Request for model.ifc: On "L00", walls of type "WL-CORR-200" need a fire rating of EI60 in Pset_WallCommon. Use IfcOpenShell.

First a look at what the model holds.

```python
import ifcopenshell
import ifcopenshell.util.element

model = ifcopenshell.open("model.ifc")
print(model.schema)
storey = next(s for s in model.by_type("IfcBuildingStorey") if s.Name == "L00")
walls = [e for e in ifcopenshell.util.element.get_decomposition(storey) if e.is_a("IfcWall")]
seen = {}
for e in walls:
    element_type = ifcopenshell.util.element.get_type(e)
    key = (element_type.Name if element_type != e and element_type else None, ifcopenshell.util.element.get_pset(e, "Pset_WallCommon", "FireRating"))
    seen[key] = seen.get(key, 0) + 1
for (name, value), count in sorted(seen.items(), key=str):
    print(count, "x", name, "|", value)
```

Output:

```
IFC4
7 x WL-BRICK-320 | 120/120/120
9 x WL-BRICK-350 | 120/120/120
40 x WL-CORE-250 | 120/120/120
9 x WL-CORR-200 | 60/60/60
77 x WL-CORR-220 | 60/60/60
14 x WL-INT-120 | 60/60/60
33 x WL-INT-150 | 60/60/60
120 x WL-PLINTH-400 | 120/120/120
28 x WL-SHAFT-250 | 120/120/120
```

```python
import ifcopenshell
import ifcopenshell.api.pset
import ifcopenshell.util.element

model = ifcopenshell.open("model.ifc")

storey = next(s for s in model.by_type("IfcBuildingStorey") if s.Name == "L00")
walls = [e for e in ifcopenshell.util.element.get_decomposition(storey) if e.is_a("IfcWall")]

count = 0
for e in walls:
    element_type = ifcopenshell.util.element.get_type(e)
    if element_type in (None, e) or element_type.Name != "WL-CORR-200":
        continue
    # add_pset returns the element's existing set when there is one.
    pset = ifcopenshell.api.pset.add_pset(model, product=e, name="Pset_WallCommon")
    ifcopenshell.api.pset.edit_pset(model, pset=pset, properties={"FireRating": "EI60"})
    count += 1

print(count, "walls updated")

model.write("model_v2.ifc")
```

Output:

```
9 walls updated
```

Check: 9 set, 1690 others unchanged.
